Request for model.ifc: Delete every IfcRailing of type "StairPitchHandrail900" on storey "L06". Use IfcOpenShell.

First a look at what the model holds.

```python
import ifcopenshell
import ifcopenshell.util.element

model = ifcopenshell.open("model.ifc")
print(model.schema)
storey = next(s for s in model.by_type("IfcBuildingStorey") if s.Name == "L06")
railings = [e for e in ifcopenshell.util.element.get_decomposition(storey) if e.is_a("IfcRailing")]
seen = {}
for e in railings:
    element_type = ifcopenshell.util.element.get_type(e)
    name = element_type.Name if element_type not in (None, e) else None
    seen[name] = seen.get(name, 0) + 1
for name, count in sorted(seen.items(), key=str):
    print(count, "x", name)
```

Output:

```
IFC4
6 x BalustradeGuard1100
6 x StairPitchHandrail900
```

```python
import ifcopenshell
import ifcopenshell.api.root
import ifcopenshell.util.element

model = ifcopenshell.open("model.ifc")

storey = next(s for s in model.by_type("IfcBuildingStorey") if s.Name == "L06")
railings = [e for e in ifcopenshell.util.element.get_decomposition(storey) if e.is_a("IfcRailing")]
targets = [e for e in railings if (t := ifcopenshell.util.element.get_type(e)) not in (None, e) and t.Name == "StairPitchHandrail900"]

for e in targets:
    ifcopenshell.api.root.remove_product(model, product=e)
print(len(targets), "removed")

model.write("model_v2.ifc")
```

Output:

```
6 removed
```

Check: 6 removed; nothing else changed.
